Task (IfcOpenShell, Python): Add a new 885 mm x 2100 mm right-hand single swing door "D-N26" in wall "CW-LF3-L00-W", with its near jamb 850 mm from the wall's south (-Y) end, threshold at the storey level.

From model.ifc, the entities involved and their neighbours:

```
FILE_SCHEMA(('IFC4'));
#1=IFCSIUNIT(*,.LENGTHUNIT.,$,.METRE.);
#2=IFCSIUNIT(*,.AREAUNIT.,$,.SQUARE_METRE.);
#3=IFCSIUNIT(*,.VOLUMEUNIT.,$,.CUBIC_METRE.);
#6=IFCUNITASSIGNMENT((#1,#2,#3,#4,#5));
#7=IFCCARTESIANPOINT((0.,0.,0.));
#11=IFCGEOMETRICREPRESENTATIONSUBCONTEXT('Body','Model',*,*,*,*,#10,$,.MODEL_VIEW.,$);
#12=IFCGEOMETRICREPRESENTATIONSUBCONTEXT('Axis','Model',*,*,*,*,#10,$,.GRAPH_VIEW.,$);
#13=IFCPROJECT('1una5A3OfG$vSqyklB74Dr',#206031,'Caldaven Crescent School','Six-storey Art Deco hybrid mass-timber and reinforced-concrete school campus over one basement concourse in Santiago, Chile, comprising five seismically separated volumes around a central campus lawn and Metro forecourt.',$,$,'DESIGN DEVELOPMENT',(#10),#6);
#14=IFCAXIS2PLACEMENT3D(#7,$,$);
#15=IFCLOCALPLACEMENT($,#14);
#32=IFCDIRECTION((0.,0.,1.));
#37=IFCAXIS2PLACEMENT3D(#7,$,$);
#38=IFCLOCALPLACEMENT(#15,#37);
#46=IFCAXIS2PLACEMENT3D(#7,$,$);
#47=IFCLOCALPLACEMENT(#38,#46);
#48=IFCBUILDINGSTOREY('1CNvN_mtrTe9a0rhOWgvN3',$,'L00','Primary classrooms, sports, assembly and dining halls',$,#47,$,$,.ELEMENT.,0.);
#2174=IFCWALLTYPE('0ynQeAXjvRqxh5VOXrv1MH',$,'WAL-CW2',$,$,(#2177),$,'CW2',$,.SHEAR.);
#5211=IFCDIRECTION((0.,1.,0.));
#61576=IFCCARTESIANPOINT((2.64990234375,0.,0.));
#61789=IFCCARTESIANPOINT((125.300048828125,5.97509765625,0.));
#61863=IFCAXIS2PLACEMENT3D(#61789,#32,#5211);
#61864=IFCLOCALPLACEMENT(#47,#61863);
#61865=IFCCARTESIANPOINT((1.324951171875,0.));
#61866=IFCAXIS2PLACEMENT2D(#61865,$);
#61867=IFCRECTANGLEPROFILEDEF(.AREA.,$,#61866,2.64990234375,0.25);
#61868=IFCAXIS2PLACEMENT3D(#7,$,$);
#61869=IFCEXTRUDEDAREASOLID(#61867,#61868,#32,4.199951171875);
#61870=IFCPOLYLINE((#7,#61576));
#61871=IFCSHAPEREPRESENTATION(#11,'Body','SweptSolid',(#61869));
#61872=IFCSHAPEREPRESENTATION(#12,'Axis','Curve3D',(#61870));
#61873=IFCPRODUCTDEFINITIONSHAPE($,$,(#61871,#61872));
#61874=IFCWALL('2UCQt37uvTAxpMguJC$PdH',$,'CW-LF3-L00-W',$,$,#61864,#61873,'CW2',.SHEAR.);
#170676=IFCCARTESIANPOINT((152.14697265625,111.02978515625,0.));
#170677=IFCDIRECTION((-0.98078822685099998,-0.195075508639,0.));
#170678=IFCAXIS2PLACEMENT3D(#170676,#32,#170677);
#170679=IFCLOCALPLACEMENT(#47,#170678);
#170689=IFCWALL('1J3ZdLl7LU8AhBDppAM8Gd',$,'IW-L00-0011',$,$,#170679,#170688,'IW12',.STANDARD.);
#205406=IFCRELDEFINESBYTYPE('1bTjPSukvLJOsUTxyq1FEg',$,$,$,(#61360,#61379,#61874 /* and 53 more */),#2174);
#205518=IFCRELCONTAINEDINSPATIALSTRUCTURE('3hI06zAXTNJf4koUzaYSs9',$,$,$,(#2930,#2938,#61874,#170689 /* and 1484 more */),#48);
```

```python
import numpy as np
import ifcopenshell
import ifcopenshell.api.feature
import ifcopenshell.api.geometry
import ifcopenshell.api.root
import ifcopenshell.api.spatial
import ifcopenshell.geom
import ifcopenshell.util.element
import ifcopenshell.util.placement
import ifcopenshell.util.representation
import ifcopenshell.util.shape
import ifcopenshell.util.unit

model = ifcopenshell.open("model.ifc")
unit_scale = ifcopenshell.util.unit.calculate_unit_scale(model)
settings = ifcopenshell.geom.settings()


def volume(element):
    """Net volume in cubic metres, openings subtracted."""
    shape = ifcopenshell.geom.create_shape(settings, element)
    return ifcopenshell.util.shape.get_volume(shape.geometry)


wall = model.by_guid("2UCQt37uvTAxpMguJC$PdH")
storey = ifcopenshell.util.element.get_container(wall, ifc_class="IfcBuildingStorey")
context = ifcopenshell.util.representation.get_context(model, "Model", "Body", "MODEL_VIEW")
before = volume(wall)

width, height, from_end, sill = 0.885, 2.1, 0.85, 0.0  # metres

# The wall runs along its own X axis, and the end named is its -X end.
wall_shape = ifcopenshell.geom.create_shape(settings, wall)
x, y, z = ifcopenshell.util.shape.get_vertices(wall_shape.geometry).T
start = x.min() + from_end
face, thickness = float(y.min()), float(y.max() - y.min())
wall_matrix = ifcopenshell.util.placement.get_local_placement(wall.ObjectPlacement)
level = ifcopenshell.util.placement.get_local_placement(storey.ObjectPlacement)[2, 3]


def in_wall(x, y):
    """Placement at x, y metres in the wall's axes, at sill height."""
    matrix = wall_matrix.copy()
    matrix[:, 3] = wall_matrix @ np.array([x / unit_scale, y / unit_scale, 0.0, 1.0])
    matrix[2, 3] = level + sill / unit_scale
    return matrix


# Opening: a box that overshoots both wall faces by 50 mm.
opening = ifcopenshell.api.root.create_entity(model, ifc_class="IfcOpeningElement", predefined_type="OPENING")
box = ifcopenshell.api.geometry.add_wall_representation(
    model, context=context, length=width, height=height, thickness=thickness + 0.1
)
ifcopenshell.api.geometry.assign_representation(model, product=opening, representation=box)
ifcopenshell.api.geometry.edit_object_placement(model, product=opening, matrix=in_wall(start, face - 0.05), is_si=False)
ifcopenshell.api.feature.add_feature(model, feature=opening, element=wall)

door = ifcopenshell.api.root.create_entity(model, ifc_class="IfcDoor", name="D-N26", predefined_type="DOOR")
door.OverallWidth, door.OverallHeight = width / unit_scale, height / unit_scale
door.OperationType = "SINGLE_SWING_RIGHT"
body = ifcopenshell.api.geometry.add_door_representation(
    model,
    context=context,
    overall_width=door.OverallWidth,
    overall_height=door.OverallHeight,
    operation_type="SINGLE_SWING_RIGHT",
    lining_properties={"LiningDepth": thickness / unit_scale, "ThresholdDepth": thickness / unit_scale},
)
ifcopenshell.api.geometry.assign_representation(model, product=door, representation=body)
ifcopenshell.api.spatial.assign_container(model, products=[door], relating_structure=storey)
ifcopenshell.api.feature.add_filling(model, opening=opening, element=door)

# The lining spans the wall, so the door starts at the wall face.
ifcopenshell.api.geometry.edit_object_placement(model, product=door, matrix=in_wall(start, face), is_si=False)

after = volume(wall)

print(f"wall volume {before:.3f} -> {after:.3f} m3")

model.write("model_v2.ifc")
```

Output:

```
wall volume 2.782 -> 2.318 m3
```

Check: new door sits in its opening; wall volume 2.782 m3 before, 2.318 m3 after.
